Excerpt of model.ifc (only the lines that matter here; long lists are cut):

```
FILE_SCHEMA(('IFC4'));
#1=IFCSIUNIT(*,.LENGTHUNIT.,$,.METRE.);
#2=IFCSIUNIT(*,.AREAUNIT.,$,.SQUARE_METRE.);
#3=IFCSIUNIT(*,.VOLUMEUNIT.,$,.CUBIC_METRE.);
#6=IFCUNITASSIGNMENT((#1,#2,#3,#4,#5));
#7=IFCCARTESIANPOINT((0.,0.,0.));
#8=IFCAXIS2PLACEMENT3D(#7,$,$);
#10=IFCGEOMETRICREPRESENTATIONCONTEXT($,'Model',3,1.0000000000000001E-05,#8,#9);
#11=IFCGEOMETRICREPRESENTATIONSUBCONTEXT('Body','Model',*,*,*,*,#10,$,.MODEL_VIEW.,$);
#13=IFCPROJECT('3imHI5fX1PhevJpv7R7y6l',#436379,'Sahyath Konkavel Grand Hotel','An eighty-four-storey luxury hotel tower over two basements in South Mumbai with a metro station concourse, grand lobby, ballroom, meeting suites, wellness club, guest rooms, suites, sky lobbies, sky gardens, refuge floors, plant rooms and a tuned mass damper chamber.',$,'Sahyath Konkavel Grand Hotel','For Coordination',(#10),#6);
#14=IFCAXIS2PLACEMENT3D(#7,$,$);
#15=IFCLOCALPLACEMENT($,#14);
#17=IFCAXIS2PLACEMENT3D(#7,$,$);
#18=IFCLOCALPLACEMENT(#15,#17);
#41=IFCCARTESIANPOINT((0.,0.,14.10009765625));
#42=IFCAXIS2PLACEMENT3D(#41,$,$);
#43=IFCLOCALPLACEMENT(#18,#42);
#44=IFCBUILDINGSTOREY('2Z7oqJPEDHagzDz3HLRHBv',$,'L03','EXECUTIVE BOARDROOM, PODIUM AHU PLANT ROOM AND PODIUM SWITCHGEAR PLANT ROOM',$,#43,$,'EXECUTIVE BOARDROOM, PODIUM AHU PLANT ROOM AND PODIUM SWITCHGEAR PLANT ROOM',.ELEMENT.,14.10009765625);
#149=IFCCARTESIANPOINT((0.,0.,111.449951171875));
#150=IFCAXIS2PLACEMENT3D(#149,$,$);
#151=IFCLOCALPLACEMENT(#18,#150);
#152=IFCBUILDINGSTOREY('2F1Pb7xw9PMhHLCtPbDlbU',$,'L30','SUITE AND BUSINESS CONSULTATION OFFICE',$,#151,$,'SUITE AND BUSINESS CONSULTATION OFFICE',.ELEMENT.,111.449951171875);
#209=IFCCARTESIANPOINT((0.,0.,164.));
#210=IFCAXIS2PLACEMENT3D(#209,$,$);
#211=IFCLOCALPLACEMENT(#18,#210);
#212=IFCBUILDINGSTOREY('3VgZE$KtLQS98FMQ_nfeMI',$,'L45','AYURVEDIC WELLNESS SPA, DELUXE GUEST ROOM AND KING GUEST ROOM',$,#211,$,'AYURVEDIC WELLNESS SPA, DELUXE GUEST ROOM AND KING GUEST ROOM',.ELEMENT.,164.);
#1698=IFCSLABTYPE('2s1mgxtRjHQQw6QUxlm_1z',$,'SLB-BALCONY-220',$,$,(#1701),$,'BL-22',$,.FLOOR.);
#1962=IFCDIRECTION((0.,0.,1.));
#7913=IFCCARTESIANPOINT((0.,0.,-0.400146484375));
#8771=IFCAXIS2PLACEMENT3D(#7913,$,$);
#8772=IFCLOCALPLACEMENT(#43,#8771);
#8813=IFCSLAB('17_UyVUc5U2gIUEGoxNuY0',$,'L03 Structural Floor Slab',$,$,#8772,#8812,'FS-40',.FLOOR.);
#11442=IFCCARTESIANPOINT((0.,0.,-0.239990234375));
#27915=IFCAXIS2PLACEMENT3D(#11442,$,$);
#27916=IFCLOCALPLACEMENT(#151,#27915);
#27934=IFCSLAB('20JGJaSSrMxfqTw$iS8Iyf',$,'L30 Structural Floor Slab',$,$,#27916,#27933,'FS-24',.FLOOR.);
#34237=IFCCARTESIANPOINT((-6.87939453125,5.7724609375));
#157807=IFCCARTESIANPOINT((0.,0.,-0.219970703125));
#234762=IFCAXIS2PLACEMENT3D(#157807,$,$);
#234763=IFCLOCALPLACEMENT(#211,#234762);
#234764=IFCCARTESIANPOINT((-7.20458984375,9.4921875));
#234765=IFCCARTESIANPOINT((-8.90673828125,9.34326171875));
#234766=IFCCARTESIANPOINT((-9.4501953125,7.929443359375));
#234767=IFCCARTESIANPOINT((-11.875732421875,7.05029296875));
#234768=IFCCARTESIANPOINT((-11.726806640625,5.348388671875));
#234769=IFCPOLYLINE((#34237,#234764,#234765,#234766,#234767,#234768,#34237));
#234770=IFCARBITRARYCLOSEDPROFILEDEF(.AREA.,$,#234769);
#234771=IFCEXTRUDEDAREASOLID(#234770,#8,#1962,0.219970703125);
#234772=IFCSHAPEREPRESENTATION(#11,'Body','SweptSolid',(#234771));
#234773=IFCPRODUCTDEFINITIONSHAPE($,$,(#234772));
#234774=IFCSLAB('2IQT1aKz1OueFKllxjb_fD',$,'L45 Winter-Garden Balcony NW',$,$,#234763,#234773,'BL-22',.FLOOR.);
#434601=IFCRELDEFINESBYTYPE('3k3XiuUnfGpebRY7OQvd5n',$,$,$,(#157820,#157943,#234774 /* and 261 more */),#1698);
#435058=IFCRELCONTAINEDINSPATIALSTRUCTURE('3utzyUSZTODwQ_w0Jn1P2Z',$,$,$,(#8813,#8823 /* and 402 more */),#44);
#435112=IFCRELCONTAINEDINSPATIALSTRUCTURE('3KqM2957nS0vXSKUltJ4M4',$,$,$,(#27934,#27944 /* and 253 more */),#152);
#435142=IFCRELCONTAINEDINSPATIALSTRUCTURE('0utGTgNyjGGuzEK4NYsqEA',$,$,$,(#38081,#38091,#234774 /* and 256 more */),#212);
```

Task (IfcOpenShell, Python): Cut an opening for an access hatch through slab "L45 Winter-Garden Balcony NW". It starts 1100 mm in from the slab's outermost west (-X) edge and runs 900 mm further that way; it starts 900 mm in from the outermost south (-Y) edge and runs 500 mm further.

```python
import numpy as np
import ifcopenshell
import ifcopenshell.api.feature
import ifcopenshell.api.geometry
import ifcopenshell.api.root
import ifcopenshell.geom
import ifcopenshell.util.placement
import ifcopenshell.util.representation
import ifcopenshell.util.shape
import ifcopenshell.util.unit

model = ifcopenshell.open("model.ifc")
unit_scale = ifcopenshell.util.unit.calculate_unit_scale(model)
settings = ifcopenshell.geom.settings()


def volume(element):
    """Net volume in cubic metres, openings subtracted."""
    shape = ifcopenshell.geom.create_shape(settings, element)
    return ifcopenshell.util.shape.get_volume(shape.geometry)


slab = model.by_guid("2IQT1aKz1OueFKllxjb_fD")
before = volume(slab)

# Extent in the slab's own axes, in metres. The edges named are its -X and -Y sides.
slab_shape = ifcopenshell.geom.create_shape(settings, slab)
vertices = ifcopenshell.util.shape.get_vertices(slab_shape.geometry)
x_min, y_min, bottom = vertices.min(axis=0)
top = vertices[:, 2].max()

opening = ifcopenshell.api.root.create_entity(model, ifc_class="IfcOpeningElement", name="Access hatch opening", predefined_type="OPENING")
context = ifcopenshell.util.representation.get_context(model, "Model", "Body", "MODEL_VIEW")
width, depth = 0.9, 0.5
outline = [(0.0, 0.0), (width, 0.0), (width, depth), (0.0, depth), (0.0, 0.0)]
# Overshoot both faces by 50 mm so the cut is clean.
shape = ifcopenshell.api.geometry.add_slab_representation(
    model, context=context, depth=top - bottom + 0.1, polyline=outline
)
ifcopenshell.api.geometry.assign_representation(model, product=opening, representation=shape)

matrix = ifcopenshell.util.placement.get_local_placement(slab.ObjectPlacement)
matrix[:, 3] = matrix @ np.append(np.array([x_min + 1.1, y_min + 0.9, bottom - 0.05]) / unit_scale, 1.0)
ifcopenshell.api.geometry.edit_object_placement(model, product=opening, matrix=matrix, is_si=False)
ifcopenshell.api.feature.add_feature(model, feature=opening, element=slab)

after = volume(slab)

print(f"slab volume {before:.3f} -> {after:.3f} m3")

model.write("model-out.ifc")
```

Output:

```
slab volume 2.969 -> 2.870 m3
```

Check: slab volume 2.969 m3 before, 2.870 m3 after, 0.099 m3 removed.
